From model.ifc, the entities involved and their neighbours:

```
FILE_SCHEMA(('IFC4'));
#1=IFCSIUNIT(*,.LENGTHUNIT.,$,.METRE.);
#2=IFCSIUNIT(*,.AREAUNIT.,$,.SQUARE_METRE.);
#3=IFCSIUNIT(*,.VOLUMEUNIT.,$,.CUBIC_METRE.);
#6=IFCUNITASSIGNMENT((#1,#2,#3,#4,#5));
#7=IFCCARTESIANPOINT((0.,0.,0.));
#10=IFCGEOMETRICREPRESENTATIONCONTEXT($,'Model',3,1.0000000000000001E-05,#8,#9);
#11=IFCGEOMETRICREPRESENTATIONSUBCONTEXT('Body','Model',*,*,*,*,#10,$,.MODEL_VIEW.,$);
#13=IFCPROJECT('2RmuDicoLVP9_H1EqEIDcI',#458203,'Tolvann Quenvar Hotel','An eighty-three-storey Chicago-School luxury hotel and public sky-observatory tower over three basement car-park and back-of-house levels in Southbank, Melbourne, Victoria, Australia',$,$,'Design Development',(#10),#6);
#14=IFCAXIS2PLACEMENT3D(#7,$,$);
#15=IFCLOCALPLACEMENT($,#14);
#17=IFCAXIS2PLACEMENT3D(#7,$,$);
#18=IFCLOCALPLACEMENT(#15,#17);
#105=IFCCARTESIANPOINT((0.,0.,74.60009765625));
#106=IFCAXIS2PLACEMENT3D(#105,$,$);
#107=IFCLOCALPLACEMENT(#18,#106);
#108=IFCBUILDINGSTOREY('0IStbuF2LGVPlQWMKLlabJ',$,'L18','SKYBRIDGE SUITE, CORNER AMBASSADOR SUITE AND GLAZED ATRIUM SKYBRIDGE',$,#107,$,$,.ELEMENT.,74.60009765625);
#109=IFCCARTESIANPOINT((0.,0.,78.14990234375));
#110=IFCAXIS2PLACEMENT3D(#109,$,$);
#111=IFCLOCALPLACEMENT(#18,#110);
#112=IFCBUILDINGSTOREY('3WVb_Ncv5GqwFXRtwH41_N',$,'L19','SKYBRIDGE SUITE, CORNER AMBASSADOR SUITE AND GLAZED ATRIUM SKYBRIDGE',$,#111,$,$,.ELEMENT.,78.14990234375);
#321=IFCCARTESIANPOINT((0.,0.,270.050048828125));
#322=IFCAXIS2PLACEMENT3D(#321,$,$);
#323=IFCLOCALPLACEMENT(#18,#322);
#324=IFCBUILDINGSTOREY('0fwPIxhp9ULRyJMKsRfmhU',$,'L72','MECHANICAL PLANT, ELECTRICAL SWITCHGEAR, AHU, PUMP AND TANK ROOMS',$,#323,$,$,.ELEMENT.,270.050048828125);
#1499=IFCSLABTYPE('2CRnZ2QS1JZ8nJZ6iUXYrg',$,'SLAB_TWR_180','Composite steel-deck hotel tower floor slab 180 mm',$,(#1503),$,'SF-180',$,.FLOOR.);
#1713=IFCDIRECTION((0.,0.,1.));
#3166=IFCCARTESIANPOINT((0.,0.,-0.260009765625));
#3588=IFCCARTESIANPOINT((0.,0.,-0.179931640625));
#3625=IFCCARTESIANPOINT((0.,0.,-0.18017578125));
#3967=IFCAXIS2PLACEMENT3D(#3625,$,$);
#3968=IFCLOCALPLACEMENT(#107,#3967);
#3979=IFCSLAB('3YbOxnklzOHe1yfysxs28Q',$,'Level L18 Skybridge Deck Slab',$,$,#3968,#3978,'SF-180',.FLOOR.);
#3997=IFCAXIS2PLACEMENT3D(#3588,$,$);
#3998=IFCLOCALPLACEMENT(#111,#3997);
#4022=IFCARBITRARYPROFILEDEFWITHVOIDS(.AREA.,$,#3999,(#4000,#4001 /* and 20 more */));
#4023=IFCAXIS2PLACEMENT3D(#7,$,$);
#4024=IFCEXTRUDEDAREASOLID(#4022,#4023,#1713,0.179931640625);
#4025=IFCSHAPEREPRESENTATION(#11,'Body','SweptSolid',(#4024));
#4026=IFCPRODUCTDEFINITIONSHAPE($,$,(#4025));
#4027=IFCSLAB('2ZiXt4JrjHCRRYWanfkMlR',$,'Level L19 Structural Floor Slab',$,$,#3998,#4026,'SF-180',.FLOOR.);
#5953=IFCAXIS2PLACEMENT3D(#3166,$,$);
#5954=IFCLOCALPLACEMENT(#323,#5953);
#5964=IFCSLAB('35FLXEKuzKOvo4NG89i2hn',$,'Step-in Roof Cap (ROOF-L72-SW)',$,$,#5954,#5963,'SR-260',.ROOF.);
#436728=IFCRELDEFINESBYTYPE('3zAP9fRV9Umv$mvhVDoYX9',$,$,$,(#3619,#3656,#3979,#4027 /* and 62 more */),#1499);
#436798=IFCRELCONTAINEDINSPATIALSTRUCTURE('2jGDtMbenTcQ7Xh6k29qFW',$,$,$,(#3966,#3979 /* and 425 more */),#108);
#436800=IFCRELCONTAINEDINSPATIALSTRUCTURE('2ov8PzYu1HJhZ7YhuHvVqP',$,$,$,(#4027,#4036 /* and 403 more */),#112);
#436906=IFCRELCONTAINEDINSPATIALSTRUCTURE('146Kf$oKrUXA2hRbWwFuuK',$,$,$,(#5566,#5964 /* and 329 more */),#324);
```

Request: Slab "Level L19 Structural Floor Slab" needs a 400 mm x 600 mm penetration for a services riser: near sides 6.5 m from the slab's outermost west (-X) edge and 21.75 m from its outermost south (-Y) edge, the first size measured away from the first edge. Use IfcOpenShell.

```python
import numpy as np
import ifcopenshell
import ifcopenshell.api.feature
import ifcopenshell.api.geometry
import ifcopenshell.api.root
import ifcopenshell.geom
import ifcopenshell.util.placement
import ifcopenshell.util.representation
import ifcopenshell.util.shape
import ifcopenshell.util.unit

model = ifcopenshell.open("model.ifc")
unit_scale = ifcopenshell.util.unit.calculate_unit_scale(model)
settings = ifcopenshell.geom.settings()


def volume(element):
    """Net volume in cubic metres, openings subtracted."""
    shape = ifcopenshell.geom.create_shape(settings, element)
    return ifcopenshell.util.shape.get_volume(shape.geometry)


slab = model.by_guid("2ZiXt4JrjHCRRYWanfkMlR")
before = volume(slab)

# Extent in the slab's own axes, in metres. The edges named are its -X and -Y sides.
slab_shape = ifcopenshell.geom.create_shape(settings, slab)
vertices = ifcopenshell.util.shape.get_vertices(slab_shape.geometry)
x_min, y_min, bottom = vertices.min(axis=0)
top = vertices[:, 2].max()

opening = ifcopenshell.api.root.create_entity(model, ifc_class="IfcOpeningElement", name="Services riser opening", predefined_type="OPENING")
context = ifcopenshell.util.representation.get_context(model, "Model", "Body", "MODEL_VIEW")
width, depth = 0.4, 0.6
outline = [(0.0, 0.0), (width, 0.0), (width, depth), (0.0, depth), (0.0, 0.0)]
# Overshoot both faces by 50 mm so the cut is clean.
shape = ifcopenshell.api.geometry.add_slab_representation(
    model, context=context, depth=top - bottom + 0.1, polyline=outline
)
ifcopenshell.api.geometry.assign_representation(model, product=opening, representation=shape)

matrix = ifcopenshell.util.placement.get_local_placement(slab.ObjectPlacement)
matrix[:, 3] = matrix @ np.append(np.array([x_min + 6.5, y_min + 21.75, bottom - 0.05]) / unit_scale, 1.0)
ifcopenshell.api.geometry.edit_object_placement(model, product=opening, matrix=matrix, is_si=False)
ifcopenshell.api.feature.add_feature(model, feature=opening, element=slab)

after = volume(slab)

print(f"slab volume {before:.3f} -> {after:.3f} m3")

model.write("model-out.ifc")
```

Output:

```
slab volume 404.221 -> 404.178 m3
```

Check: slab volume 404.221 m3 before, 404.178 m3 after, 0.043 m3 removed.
